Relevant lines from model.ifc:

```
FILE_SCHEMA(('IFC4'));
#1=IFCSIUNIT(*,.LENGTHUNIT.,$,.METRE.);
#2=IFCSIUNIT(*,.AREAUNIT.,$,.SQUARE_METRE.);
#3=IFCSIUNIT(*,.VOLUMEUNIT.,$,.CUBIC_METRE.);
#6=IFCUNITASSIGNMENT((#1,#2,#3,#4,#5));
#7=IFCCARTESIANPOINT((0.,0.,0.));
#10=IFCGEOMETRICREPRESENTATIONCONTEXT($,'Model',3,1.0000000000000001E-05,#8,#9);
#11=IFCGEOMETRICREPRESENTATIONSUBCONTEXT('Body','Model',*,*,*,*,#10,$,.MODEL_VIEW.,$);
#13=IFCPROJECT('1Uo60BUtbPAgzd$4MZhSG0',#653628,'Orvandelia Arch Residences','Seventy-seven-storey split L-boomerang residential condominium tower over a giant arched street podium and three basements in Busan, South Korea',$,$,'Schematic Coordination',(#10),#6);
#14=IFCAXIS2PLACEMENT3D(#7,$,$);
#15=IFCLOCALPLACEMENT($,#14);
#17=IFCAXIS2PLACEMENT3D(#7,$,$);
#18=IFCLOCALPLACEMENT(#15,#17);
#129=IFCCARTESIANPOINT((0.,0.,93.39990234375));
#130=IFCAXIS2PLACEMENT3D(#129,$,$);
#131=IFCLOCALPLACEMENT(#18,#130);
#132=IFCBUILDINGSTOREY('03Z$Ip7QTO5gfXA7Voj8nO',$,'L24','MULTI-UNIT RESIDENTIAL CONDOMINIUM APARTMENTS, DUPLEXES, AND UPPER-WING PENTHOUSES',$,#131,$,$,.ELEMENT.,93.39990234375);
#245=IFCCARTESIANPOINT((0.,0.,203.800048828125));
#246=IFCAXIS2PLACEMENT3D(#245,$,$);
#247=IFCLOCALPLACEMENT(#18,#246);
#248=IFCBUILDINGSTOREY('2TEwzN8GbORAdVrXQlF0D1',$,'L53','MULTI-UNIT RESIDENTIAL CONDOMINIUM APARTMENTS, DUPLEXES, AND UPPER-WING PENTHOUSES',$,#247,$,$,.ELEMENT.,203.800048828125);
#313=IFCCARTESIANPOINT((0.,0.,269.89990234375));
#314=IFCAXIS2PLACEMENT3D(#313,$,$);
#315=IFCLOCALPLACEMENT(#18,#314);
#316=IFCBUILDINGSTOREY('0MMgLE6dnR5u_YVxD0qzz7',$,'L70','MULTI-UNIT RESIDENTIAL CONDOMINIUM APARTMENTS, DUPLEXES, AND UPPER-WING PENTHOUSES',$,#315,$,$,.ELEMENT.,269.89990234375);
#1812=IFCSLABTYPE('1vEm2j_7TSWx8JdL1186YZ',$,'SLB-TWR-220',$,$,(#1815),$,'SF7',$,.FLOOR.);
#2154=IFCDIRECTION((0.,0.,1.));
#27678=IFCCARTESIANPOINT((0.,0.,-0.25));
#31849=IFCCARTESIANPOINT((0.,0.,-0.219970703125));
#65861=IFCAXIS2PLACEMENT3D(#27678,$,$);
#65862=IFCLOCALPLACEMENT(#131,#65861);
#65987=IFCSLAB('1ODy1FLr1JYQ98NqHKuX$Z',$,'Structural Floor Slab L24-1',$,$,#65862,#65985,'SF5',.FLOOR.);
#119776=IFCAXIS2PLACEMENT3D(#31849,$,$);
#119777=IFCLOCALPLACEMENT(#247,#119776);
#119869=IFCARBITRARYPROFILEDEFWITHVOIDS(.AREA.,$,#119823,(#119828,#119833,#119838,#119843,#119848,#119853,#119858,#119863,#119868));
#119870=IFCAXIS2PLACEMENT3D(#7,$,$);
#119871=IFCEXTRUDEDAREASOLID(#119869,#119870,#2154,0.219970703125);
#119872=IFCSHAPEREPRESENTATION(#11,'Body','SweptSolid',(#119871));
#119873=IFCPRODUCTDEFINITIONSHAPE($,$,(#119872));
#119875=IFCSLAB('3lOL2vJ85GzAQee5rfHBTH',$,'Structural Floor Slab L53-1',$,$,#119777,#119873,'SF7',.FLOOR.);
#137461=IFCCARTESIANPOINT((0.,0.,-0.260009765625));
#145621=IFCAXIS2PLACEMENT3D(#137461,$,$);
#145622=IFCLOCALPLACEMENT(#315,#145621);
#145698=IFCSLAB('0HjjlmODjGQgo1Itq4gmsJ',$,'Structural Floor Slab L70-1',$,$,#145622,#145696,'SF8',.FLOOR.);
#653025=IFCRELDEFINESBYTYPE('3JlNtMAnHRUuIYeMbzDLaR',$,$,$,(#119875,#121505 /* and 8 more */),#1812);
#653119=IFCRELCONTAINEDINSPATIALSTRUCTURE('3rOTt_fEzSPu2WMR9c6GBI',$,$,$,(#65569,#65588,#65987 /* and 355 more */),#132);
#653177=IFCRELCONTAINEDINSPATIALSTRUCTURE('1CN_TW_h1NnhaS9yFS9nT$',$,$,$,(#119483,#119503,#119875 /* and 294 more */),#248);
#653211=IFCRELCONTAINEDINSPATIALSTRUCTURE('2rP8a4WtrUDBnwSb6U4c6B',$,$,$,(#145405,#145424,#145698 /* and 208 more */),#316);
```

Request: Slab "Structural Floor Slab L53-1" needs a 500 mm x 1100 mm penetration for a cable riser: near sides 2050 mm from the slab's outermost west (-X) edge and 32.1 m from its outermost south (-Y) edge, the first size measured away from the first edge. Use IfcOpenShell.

```python
import numpy as np
import ifcopenshell
import ifcopenshell.api.feature
import ifcopenshell.api.geometry
import ifcopenshell.api.root
import ifcopenshell.geom
import ifcopenshell.util.placement
import ifcopenshell.util.representation
import ifcopenshell.util.shape
import ifcopenshell.util.unit

model = ifcopenshell.open("model.ifc")
unit_scale = ifcopenshell.util.unit.calculate_unit_scale(model)
settings = ifcopenshell.geom.settings()


def volume(element):
    """Net volume in cubic metres, openings subtracted."""
    shape = ifcopenshell.geom.create_shape(settings, element)
    return ifcopenshell.util.shape.get_volume(shape.geometry)


slab = model.by_guid("3lOL2vJ85GzAQee5rfHBTH")
before = volume(slab)

# Extent in the slab's own axes, in metres. The edges named are its -X and -Y sides.
slab_shape = ifcopenshell.geom.create_shape(settings, slab)
vertices = ifcopenshell.util.shape.get_vertices(slab_shape.geometry)
x_min, y_min, bottom = vertices.min(axis=0)
top = vertices[:, 2].max()

opening = ifcopenshell.api.root.create_entity(model, ifc_class="IfcOpeningElement", name="Cable riser opening", predefined_type="OPENING")
context = ifcopenshell.util.representation.get_context(model, "Model", "Body", "MODEL_VIEW")
width, depth = 0.5, 1.1
outline = [(0.0, 0.0), (width, 0.0), (width, depth), (0.0, depth), (0.0, 0.0)]
# Overshoot both faces by 50 mm so the cut is clean.
shape = ifcopenshell.api.geometry.add_slab_representation(
    model, context=context, depth=top - bottom + 0.1, polyline=outline
)
ifcopenshell.api.geometry.assign_representation(model, product=opening, representation=shape)

matrix = ifcopenshell.util.placement.get_local_placement(slab.ObjectPlacement)
matrix[:, 3] = matrix @ np.append(np.array([x_min + 2.05, y_min + 32.1, bottom - 0.05]) / unit_scale, 1.0)
ifcopenshell.api.geometry.edit_object_placement(model, product=opening, matrix=matrix, is_si=False)
ifcopenshell.api.feature.add_feature(model, feature=opening, element=slab)

after = volume(slab)

print(f"slab volume {before:.3f} -> {after:.3f} m3")

model.write("model_edited.ifc")
```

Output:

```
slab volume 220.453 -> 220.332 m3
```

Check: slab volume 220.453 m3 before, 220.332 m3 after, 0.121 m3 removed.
